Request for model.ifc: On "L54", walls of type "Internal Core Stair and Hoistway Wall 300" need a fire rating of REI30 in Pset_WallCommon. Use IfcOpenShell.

First a look at what the model holds.

```python
import ifcopenshell
import ifcopenshell.util.element

model = ifcopenshell.open("model.ifc")
print(model.schema)
storey = next(s for s in model.by_type("IfcBuildingStorey") if s.Name == "L54")
walls = [e for e in ifcopenshell.util.element.get_decomposition(storey) if e.is_a("IfcWall")]
seen = {}
for e in walls:
    element_type = ifcopenshell.util.element.get_type(e)
    key = (element_type.Name if element_type != e and element_type else None, ifcopenshell.util.element.get_pset(e, "Pset_WallCommon", "FireRating"))
    seen[key] = seen.get(key, 0) + 1
for (name, value), count in sorted(seen.items(), key=str):
    print(count, "x", name, "|", value)
```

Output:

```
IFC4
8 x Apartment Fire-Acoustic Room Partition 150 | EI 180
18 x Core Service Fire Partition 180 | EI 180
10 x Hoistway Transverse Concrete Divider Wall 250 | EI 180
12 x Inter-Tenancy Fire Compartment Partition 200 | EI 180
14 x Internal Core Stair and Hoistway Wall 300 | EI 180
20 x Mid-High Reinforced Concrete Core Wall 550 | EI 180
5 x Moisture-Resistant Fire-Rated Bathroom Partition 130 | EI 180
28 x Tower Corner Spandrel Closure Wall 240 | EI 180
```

```python
import ifcopenshell
import ifcopenshell.api.pset
import ifcopenshell.util.element

model = ifcopenshell.open("model.ifc")

storey = next(s for s in model.by_type("IfcBuildingStorey") if s.Name == "L54")
walls = [e for e in ifcopenshell.util.element.get_decomposition(storey) if e.is_a("IfcWall")]

count = 0
for e in walls:
    element_type = ifcopenshell.util.element.get_type(e)
    if element_type in (None, e) or element_type.Name != "Internal Core Stair and Hoistway Wall 300":
        continue
    found = ifcopenshell.util.element.get_pset(e, "Pset_WallCommon", should_inherit=False)
    if found:
        pset = model.by_id(found["id"])
        if len(ifcopenshell.util.element.get_elements_by_pset(pset)) > 1:
            pset = ifcopenshell.api.pset.unshare_pset(model, products=[e], pset=pset)[0]
    else:
        pset = ifcopenshell.api.pset.add_pset(model, product=e, name="Pset_WallCommon")
    ifcopenshell.api.pset.edit_pset(model, pset=pset, properties={"FireRating": "REI30"})
    count += 1

print(count, "walls updated")

model.write("model_updated.ifc")
```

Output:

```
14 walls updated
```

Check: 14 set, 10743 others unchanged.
